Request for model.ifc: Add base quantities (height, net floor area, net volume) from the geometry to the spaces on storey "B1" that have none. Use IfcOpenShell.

First a look at what the model holds.

```python
import ifcopenshell
import ifcopenshell.util.element
import ifcopenshell.util.unit

model = ifcopenshell.open("model.ifc")
print(model.schema)
for unit_type in ("LENGTHUNIT", "AREAUNIT", "VOLUMEUNIT"):
    print(unit_type, ifcopenshell.util.unit.calculate_unit_scale(model, unit_type))
storey = next(s for s in model.by_type("IfcBuildingStorey") if s.Name == "B1")
spaces = [e for e in ifcopenshell.util.element.get_decomposition(storey) if e.is_a("IfcSpace")]
for e in sorted(spaces, key=lambda e: e.id()):
    print(e.id(), e.is_a(), e.Name, list(ifcopenshell.util.element.get_psets(e, qtos_only=True)), sep=" | ")
```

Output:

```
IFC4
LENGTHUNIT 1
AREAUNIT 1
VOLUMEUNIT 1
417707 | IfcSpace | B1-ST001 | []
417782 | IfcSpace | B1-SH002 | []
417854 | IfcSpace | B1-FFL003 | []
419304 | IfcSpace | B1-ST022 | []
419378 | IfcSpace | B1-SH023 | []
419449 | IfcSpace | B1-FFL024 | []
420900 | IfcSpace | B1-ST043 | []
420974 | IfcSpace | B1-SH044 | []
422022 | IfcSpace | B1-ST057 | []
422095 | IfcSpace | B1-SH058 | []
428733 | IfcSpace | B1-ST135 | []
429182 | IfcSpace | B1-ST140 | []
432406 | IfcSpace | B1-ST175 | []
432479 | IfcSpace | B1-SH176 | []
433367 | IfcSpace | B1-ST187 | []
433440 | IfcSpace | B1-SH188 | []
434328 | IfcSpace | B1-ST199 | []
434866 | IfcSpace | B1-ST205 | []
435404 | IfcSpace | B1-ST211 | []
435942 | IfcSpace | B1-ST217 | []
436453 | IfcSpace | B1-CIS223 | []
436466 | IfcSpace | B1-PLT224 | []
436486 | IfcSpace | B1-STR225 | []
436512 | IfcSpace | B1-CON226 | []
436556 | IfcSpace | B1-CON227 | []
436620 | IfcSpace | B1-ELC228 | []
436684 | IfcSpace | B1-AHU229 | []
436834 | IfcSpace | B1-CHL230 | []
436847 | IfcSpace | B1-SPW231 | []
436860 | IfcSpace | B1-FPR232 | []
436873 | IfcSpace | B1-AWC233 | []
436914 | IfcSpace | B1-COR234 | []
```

```python
import ifcopenshell
import ifcopenshell.api.pset
import ifcopenshell.geom
import ifcopenshell.util.element
import ifcopenshell.util.shape
import ifcopenshell.util.unit

model = ifcopenshell.open("model.ifc")
unit_scale = ifcopenshell.util.unit.calculate_unit_scale(model)
area_scale = ifcopenshell.util.unit.calculate_unit_scale(model, "AREAUNIT")
volume_scale = ifcopenshell.util.unit.calculate_unit_scale(model, "VOLUMEUNIT")
settings = ifcopenshell.geom.settings()

storey = next(s for s in model.by_type("IfcBuildingStorey") if s.Name == "B1")
spaces = [e for e in ifcopenshell.util.element.get_decomposition(storey) if e.is_a("IfcSpace")]

for e in sorted(spaces, key=lambda e: e.id()):
    if ifcopenshell.util.element.get_psets(e, qtos_only=True, should_inherit=False):
        continue
    # Geometry comes back in metres, in the element's own axes.
    shape = ifcopenshell.geom.create_shape(settings, e)
    values = {
        "Height": ifcopenshell.util.shape.get_z(shape.geometry) / unit_scale,
        "NetFloorArea": ifcopenshell.util.shape.get_footprint_area(shape.geometry) / area_scale,
        "NetVolume": ifcopenshell.util.shape.get_volume(shape.geometry) / volume_scale,
    }
    qto = ifcopenshell.api.pset.add_qto(model, product=e, name="Qto_SpaceBaseQuantities")
    ifcopenshell.api.pset.edit_qto(model, qto=qto, properties=values)
    print(e.id(), {k: round(v, 3) for k, v in values.items()})

model.write("model_edited.ifc")
```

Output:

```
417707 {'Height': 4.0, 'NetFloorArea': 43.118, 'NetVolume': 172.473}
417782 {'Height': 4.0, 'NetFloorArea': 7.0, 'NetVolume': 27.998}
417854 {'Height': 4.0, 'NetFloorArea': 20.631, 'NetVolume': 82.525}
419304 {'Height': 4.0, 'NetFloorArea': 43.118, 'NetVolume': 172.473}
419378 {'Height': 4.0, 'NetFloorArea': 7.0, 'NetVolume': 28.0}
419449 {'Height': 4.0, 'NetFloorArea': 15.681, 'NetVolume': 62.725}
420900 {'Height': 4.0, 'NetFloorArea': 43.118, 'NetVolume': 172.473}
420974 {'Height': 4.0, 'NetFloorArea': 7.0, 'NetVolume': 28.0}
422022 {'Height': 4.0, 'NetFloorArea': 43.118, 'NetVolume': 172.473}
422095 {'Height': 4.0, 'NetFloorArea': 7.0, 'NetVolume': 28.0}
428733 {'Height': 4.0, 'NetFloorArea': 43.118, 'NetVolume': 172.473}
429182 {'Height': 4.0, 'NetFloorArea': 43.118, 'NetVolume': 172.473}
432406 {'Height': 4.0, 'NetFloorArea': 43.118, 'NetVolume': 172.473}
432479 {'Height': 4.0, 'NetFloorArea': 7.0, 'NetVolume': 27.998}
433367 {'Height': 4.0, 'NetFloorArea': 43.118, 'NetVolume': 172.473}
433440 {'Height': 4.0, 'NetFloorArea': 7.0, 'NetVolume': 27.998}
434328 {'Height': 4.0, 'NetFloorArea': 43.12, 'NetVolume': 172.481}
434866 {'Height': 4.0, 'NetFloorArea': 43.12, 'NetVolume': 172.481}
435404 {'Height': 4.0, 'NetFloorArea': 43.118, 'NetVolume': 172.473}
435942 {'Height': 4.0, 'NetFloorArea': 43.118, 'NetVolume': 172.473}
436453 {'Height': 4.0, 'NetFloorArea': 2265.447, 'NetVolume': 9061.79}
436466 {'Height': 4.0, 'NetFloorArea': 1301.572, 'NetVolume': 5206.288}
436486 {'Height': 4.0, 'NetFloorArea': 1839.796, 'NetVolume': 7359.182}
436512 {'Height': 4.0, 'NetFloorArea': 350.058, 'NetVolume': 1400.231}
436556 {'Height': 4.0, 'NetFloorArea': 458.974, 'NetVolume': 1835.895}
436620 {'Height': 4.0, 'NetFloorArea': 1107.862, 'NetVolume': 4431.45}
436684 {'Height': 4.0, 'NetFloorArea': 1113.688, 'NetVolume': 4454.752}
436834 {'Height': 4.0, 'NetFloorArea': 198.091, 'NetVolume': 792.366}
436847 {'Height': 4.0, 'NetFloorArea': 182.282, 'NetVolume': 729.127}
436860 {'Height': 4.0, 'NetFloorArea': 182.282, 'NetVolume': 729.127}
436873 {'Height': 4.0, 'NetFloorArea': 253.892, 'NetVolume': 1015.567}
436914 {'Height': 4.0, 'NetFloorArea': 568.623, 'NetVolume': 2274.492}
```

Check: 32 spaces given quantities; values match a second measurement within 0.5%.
